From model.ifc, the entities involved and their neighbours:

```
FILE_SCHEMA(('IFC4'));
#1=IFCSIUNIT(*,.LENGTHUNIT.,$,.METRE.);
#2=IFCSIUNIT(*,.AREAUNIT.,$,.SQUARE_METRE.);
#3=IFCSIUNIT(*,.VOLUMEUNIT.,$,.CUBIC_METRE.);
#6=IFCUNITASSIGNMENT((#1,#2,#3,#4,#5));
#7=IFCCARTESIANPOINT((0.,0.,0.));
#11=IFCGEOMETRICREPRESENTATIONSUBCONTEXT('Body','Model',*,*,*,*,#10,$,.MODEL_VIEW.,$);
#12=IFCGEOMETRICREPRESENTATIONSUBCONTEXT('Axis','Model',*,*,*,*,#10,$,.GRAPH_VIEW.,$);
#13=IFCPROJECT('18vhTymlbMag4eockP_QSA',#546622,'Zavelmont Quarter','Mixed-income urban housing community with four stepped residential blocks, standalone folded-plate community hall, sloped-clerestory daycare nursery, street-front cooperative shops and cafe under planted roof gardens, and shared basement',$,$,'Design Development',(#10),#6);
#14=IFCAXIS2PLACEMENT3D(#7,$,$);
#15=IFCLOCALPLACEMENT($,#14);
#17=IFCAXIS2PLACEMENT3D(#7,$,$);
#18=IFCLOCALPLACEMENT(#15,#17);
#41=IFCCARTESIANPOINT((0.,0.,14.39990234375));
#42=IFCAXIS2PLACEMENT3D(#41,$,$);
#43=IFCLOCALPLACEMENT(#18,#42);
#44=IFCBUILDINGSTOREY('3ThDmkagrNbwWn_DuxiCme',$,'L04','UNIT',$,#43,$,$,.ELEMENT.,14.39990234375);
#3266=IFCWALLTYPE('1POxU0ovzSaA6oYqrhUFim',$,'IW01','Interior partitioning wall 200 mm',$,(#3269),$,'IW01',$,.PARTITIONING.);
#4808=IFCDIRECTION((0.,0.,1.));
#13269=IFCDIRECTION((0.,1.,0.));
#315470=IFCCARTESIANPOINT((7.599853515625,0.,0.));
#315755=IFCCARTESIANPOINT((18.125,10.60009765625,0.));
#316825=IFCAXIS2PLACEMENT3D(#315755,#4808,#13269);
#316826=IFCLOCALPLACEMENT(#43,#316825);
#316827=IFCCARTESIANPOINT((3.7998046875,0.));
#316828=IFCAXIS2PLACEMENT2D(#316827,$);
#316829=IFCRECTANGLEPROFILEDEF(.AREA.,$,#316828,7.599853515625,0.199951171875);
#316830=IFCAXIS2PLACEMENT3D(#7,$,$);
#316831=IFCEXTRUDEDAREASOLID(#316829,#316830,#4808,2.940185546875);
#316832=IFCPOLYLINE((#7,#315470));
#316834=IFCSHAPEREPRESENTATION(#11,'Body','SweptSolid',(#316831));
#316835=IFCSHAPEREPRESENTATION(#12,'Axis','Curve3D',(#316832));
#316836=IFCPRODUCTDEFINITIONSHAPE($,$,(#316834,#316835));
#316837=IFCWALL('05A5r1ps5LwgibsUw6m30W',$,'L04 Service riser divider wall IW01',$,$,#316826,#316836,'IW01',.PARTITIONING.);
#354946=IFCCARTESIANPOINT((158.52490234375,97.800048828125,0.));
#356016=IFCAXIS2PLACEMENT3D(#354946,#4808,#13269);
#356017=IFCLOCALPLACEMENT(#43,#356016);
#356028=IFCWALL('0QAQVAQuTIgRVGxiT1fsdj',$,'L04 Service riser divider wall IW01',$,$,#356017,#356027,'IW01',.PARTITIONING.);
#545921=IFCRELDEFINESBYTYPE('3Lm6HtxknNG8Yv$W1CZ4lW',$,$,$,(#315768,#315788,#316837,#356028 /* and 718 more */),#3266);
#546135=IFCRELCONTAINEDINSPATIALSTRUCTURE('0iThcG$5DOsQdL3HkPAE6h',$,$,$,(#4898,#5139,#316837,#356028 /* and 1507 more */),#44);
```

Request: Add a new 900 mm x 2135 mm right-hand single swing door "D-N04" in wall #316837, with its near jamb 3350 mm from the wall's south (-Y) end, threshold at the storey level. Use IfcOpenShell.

```python
import numpy as np
import ifcopenshell
import ifcopenshell.api.feature
import ifcopenshell.api.geometry
import ifcopenshell.api.root
import ifcopenshell.api.spatial
import ifcopenshell.geom
import ifcopenshell.util.element
import ifcopenshell.util.placement
import ifcopenshell.util.representation
import ifcopenshell.util.shape
import ifcopenshell.util.unit

model = ifcopenshell.open("model.ifc")
unit_scale = ifcopenshell.util.unit.calculate_unit_scale(model)
settings = ifcopenshell.geom.settings()


def volume(element):
    """Net volume in cubic metres, openings subtracted."""
    shape = ifcopenshell.geom.create_shape(settings, element)
    return ifcopenshell.util.shape.get_volume(shape.geometry)


wall = model.by_guid("05A5r1ps5LwgibsUw6m30W")
storey = ifcopenshell.util.element.get_container(wall, ifc_class="IfcBuildingStorey")
context = ifcopenshell.util.representation.get_context(model, "Model", "Body", "MODEL_VIEW")
before = volume(wall)

width, height, from_end, sill = 0.9, 2.135, 3.35, 0.0  # metres

# The wall runs along its own X axis, and the end named is its -X end.
wall_shape = ifcopenshell.geom.create_shape(settings, wall)
x, y, z = ifcopenshell.util.shape.get_vertices(wall_shape.geometry).T
start = x.min() + from_end
face, thickness = float(y.min()), float(y.max() - y.min())
wall_matrix = ifcopenshell.util.placement.get_local_placement(wall.ObjectPlacement)
level = ifcopenshell.util.placement.get_local_placement(storey.ObjectPlacement)[2, 3]


def in_wall(x, y):
    """Placement at x, y metres in the wall's axes, at sill height."""
    matrix = wall_matrix.copy()
    matrix[:, 3] = wall_matrix @ np.array([x / unit_scale, y / unit_scale, 0.0, 1.0])
    matrix[2, 3] = level + sill / unit_scale
    return matrix


# Opening: a box that overshoots both wall faces by 50 mm.
opening = ifcopenshell.api.root.create_entity(model, ifc_class="IfcOpeningElement", predefined_type="OPENING")
box = ifcopenshell.api.geometry.add_wall_representation(
    model, context=context, length=width, height=height, thickness=thickness + 0.1
)
ifcopenshell.api.geometry.assign_representation(model, product=opening, representation=box)
ifcopenshell.api.geometry.edit_object_placement(model, product=opening, matrix=in_wall(start, face - 0.05), is_si=False)
ifcopenshell.api.feature.add_feature(model, feature=opening, element=wall)

door = ifcopenshell.api.root.create_entity(model, ifc_class="IfcDoor", name="D-N04", predefined_type="DOOR")
door.OverallWidth, door.OverallHeight = width / unit_scale, height / unit_scale
door.OperationType = "SINGLE_SWING_RIGHT"
body = ifcopenshell.api.geometry.add_door_representation(
    model,
    context=context,
    overall_width=door.OverallWidth,
    overall_height=door.OverallHeight,
    operation_type="SINGLE_SWING_RIGHT",
    lining_properties={"LiningDepth": thickness / unit_scale, "ThresholdDepth": thickness / unit_scale},
)
ifcopenshell.api.geometry.assign_representation(model, product=door, representation=body)
ifcopenshell.api.spatial.assign_container(model, products=[door], relating_structure=storey)
ifcopenshell.api.feature.add_filling(model, opening=opening, element=door)

# The lining spans the wall, so the door starts at the wall face.
ifcopenshell.api.geometry.edit_object_placement(model, product=door, matrix=in_wall(start, face), is_si=False)

after = volume(wall)

print(f"wall volume {before:.3f} -> {after:.3f} m3")

model.write("model_edited.ifc")
```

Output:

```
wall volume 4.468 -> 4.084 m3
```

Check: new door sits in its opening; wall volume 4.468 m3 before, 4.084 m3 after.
